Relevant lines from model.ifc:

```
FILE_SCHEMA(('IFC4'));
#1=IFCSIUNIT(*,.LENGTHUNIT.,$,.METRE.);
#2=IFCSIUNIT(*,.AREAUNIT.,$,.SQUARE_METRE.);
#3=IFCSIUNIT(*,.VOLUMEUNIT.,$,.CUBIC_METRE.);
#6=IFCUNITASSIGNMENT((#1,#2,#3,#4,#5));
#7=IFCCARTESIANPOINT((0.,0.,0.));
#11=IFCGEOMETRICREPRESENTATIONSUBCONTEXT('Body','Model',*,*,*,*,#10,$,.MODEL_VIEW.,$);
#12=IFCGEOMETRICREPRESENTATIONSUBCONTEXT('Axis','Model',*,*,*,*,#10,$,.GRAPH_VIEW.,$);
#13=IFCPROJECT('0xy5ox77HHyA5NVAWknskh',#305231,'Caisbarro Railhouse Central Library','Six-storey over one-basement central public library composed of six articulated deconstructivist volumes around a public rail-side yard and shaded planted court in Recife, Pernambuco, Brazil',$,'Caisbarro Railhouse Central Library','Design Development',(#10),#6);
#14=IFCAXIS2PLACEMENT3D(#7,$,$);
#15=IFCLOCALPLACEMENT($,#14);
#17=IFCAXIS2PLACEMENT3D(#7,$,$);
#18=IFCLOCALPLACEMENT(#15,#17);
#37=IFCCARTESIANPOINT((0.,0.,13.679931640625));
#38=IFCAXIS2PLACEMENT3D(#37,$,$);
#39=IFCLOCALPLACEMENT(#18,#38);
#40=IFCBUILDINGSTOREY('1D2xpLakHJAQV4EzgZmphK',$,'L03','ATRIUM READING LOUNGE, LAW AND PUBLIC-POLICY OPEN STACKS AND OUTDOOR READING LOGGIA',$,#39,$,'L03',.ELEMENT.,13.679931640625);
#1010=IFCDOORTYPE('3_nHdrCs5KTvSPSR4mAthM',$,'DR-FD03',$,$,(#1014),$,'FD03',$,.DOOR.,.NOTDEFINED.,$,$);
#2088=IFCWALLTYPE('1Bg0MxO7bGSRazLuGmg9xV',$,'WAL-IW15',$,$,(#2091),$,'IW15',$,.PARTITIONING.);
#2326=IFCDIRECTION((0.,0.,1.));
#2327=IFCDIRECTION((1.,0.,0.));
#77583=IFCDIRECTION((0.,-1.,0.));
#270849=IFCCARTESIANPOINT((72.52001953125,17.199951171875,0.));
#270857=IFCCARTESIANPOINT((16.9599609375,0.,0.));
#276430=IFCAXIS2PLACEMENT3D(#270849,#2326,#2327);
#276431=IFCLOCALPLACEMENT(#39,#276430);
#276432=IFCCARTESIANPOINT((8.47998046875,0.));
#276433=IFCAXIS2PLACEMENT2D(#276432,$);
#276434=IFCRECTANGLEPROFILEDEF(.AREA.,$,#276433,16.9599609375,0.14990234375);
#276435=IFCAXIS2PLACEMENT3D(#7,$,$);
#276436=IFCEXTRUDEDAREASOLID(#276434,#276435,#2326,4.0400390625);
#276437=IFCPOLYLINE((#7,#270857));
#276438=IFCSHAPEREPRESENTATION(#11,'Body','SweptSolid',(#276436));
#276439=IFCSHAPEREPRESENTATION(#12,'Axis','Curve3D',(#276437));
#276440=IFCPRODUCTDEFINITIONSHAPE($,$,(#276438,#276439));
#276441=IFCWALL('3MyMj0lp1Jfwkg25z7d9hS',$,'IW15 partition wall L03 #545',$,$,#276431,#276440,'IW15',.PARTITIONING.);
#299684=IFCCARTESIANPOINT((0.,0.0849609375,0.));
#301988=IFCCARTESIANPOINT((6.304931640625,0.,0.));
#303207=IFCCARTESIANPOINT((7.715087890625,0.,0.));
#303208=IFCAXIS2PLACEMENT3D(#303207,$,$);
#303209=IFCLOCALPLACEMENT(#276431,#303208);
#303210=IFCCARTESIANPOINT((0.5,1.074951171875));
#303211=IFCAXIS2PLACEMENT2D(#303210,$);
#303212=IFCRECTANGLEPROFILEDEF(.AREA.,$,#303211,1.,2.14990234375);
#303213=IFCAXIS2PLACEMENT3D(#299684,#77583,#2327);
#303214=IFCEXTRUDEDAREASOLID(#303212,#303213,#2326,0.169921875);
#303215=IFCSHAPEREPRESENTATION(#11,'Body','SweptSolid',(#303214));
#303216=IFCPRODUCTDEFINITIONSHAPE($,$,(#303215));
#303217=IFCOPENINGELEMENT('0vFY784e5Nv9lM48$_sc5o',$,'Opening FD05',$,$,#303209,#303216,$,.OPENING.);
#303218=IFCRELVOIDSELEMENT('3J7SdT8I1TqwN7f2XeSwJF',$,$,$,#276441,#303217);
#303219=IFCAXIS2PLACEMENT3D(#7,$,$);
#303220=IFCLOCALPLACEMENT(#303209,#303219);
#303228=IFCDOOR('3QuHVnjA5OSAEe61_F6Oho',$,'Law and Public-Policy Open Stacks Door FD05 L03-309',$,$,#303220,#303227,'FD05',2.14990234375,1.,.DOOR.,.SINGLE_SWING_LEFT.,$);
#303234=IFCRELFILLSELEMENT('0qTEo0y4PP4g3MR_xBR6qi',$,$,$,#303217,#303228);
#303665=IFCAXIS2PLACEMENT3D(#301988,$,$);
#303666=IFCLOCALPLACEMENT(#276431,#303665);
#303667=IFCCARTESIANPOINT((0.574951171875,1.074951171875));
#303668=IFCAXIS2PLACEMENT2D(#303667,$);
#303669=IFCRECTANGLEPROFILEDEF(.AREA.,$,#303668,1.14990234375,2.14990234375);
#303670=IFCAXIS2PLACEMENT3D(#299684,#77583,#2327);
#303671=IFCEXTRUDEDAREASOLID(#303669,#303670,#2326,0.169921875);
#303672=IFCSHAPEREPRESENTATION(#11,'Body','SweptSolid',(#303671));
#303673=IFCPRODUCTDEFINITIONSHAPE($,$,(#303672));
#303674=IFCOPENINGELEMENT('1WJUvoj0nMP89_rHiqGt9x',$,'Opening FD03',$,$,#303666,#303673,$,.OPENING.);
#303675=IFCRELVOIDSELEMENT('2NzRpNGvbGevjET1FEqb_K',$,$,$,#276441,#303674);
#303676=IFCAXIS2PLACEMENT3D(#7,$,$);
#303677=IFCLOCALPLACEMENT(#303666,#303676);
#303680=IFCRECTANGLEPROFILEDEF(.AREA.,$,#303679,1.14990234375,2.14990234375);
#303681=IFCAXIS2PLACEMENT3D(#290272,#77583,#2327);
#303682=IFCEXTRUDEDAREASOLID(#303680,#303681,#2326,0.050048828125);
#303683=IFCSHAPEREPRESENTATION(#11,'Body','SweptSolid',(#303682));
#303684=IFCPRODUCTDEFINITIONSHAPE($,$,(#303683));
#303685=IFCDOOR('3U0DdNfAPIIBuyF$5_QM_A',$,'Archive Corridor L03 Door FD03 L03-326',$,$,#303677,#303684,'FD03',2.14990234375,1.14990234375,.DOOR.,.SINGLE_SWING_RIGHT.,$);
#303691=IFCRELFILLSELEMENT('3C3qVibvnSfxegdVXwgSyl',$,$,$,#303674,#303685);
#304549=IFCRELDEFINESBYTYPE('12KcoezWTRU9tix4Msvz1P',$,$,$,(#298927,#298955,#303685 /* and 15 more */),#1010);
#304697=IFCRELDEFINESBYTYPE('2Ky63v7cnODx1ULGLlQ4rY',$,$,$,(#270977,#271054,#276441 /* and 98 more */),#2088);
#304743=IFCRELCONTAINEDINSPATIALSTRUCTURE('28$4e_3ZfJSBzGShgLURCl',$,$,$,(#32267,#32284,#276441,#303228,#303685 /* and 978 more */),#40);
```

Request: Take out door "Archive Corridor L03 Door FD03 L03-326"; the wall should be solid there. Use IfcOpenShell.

```python
import ifcopenshell
import ifcopenshell.api.feature
import ifcopenshell.api.root
import ifcopenshell.geom
import ifcopenshell.util.shape

model = ifcopenshell.open("model.ifc")
settings = ifcopenshell.geom.settings()


def volume(element):
    """Net volume in cubic metres, openings subtracted."""
    shape = ifcopenshell.geom.create_shape(settings, element)
    return ifcopenshell.util.shape.get_volume(shape.geometry)


door = model.by_guid("3U0DdNfAPIIBuyF$5_QM_A")
opening = door.FillsVoids[0].RelatingOpeningElement
wall = opening.VoidsElements[0].RelatingBuildingElement
before = volume(wall)

ifcopenshell.api.root.remove_product(model, product=door)
ifcopenshell.api.feature.remove_feature(model, feature=opening)

after = volume(wall)

print(f"wall volume {before:.3f} -> {after:.3f} m3")

model.write("model_edited.ifc")
```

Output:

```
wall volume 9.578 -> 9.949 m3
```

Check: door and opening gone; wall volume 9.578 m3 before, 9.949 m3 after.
